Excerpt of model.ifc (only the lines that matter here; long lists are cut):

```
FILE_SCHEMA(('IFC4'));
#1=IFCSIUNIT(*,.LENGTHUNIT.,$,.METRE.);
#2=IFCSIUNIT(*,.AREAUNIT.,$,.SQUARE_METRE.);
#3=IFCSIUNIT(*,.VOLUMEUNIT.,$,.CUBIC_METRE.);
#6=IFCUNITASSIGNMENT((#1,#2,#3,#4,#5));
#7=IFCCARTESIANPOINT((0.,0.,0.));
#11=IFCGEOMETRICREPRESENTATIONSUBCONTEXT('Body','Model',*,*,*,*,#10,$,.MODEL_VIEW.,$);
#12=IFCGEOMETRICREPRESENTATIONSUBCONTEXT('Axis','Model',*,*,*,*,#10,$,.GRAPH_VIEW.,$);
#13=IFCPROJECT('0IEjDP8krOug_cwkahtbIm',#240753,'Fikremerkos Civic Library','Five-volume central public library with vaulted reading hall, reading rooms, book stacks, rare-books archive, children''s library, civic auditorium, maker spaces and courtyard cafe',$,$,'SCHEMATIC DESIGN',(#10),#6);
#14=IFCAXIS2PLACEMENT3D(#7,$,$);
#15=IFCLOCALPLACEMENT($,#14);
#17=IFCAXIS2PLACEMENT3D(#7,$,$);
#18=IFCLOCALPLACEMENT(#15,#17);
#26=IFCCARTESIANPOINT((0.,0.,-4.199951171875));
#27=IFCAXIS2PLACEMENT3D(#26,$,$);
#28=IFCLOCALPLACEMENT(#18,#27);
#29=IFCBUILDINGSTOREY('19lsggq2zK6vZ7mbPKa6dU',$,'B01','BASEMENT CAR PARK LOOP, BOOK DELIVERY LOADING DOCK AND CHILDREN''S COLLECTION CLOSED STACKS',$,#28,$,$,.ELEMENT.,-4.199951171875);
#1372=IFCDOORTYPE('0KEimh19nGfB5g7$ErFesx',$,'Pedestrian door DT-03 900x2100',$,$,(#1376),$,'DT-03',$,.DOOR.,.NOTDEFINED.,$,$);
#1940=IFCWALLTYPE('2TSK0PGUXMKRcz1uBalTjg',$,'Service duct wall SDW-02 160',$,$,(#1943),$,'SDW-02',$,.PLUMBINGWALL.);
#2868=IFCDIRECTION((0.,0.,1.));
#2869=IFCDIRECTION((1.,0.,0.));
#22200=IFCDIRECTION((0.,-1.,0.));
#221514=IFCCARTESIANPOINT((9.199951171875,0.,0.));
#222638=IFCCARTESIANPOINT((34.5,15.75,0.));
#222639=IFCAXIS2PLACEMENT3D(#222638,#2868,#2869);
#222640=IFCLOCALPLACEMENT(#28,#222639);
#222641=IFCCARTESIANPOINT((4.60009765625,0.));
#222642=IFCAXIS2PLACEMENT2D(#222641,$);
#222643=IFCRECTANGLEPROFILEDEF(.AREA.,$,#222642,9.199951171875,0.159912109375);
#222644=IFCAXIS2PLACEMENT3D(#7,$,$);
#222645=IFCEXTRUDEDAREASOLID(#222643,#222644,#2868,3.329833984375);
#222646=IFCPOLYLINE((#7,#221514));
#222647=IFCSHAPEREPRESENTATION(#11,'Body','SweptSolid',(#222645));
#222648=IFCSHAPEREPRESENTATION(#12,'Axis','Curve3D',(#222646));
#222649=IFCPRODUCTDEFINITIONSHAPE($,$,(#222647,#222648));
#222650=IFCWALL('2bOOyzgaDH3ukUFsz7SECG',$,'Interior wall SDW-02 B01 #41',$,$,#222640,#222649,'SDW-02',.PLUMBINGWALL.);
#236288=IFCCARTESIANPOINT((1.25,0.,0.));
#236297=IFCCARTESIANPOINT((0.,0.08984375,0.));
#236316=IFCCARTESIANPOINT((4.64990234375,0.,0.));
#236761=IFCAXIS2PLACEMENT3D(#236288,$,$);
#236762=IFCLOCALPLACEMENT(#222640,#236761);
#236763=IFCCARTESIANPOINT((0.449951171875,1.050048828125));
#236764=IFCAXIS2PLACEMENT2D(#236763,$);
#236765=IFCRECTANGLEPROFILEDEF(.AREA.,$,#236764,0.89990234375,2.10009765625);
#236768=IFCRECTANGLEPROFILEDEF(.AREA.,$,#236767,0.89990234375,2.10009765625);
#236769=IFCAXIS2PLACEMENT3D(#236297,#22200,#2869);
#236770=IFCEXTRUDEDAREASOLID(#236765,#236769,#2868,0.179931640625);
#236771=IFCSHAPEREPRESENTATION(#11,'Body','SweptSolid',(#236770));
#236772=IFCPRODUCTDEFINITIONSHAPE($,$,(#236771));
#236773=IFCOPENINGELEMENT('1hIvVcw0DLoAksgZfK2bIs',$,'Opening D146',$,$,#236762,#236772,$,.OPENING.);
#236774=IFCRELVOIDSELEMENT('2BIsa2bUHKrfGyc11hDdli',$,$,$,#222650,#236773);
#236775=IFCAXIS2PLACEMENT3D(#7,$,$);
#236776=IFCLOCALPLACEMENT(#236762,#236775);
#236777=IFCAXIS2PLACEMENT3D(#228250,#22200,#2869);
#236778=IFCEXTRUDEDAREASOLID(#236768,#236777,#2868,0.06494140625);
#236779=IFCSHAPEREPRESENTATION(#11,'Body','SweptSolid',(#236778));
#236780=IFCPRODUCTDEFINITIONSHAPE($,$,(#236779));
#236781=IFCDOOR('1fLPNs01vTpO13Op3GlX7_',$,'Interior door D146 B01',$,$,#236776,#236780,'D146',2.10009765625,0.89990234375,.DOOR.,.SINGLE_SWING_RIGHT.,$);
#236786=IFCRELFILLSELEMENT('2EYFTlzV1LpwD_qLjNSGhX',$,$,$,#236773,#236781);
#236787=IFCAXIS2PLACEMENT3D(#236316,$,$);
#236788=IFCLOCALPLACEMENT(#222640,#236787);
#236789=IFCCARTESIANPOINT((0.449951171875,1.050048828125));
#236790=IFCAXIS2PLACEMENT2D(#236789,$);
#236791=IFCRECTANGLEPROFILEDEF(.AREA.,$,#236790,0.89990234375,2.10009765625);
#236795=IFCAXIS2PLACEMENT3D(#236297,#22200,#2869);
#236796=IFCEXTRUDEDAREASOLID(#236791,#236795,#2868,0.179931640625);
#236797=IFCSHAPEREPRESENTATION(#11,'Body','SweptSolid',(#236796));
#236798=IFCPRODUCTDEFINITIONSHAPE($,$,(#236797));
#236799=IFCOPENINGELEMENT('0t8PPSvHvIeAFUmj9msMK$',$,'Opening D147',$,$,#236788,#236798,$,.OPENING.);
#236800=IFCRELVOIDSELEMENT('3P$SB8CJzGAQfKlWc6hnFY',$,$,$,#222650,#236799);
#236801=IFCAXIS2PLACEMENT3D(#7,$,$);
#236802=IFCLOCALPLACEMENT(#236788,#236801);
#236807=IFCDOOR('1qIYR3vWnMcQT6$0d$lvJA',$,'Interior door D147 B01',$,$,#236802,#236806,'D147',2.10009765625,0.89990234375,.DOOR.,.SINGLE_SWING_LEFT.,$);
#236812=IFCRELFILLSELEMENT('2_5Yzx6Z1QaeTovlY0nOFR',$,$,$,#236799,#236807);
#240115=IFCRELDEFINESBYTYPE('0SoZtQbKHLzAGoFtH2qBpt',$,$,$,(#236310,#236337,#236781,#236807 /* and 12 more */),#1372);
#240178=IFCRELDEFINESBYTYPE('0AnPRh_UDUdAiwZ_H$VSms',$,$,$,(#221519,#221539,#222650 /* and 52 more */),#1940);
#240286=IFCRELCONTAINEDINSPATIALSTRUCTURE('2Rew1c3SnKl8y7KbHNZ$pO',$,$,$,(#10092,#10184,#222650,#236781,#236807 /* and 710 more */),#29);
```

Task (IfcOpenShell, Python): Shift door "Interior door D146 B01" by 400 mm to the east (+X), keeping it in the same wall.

```python
import ifcopenshell
import ifcopenshell.api.geometry
import ifcopenshell.util.placement

model = ifcopenshell.open("model.ifc")

door = model.by_guid("1fLPNs01vTpO13Op3GlX7_")
opening = door.FillsVoids[0].RelatingOpeningElement
wall = opening.VoidsElements[0].RelatingBuildingElement

wall_matrix = ifcopenshell.util.placement.get_local_placement(wall.ObjectPlacement)
shift = wall_matrix[:3, 0] * 0.4
before = ifcopenshell.util.placement.get_local_placement(door.ObjectPlacement)[:3, 3].copy()

# The door is placed relative to its opening, so it follows when the opening moves.
matrix = ifcopenshell.util.placement.get_local_placement(opening.ObjectPlacement)
matrix[:3, 3] += shift
ifcopenshell.api.geometry.edit_object_placement(
    model, product=opening, matrix=matrix, is_si=False, should_transform_children=True
)

after = ifcopenshell.util.placement.get_local_placement(door.ObjectPlacement)[:3, 3]
print("door moved by", (after - before).round(3) + 0.0)

model.write("model_edited.ifc")
```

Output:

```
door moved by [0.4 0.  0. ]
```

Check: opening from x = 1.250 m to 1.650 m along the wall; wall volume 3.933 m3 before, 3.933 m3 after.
